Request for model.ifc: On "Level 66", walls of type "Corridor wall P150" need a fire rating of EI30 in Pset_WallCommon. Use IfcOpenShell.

First a look at what the model holds.

```python
import ifcopenshell
import ifcopenshell.util.element

model = ifcopenshell.open("model.ifc")
print(model.schema)
storey = next(s for s in model.by_type("IfcBuildingStorey") if s.Name == "Level 66")
walls = [e for e in ifcopenshell.util.element.get_decomposition(storey) if e.is_a("IfcWall")]
seen = {}
for e in walls:
    element_type = ifcopenshell.util.element.get_type(e)
    key = (element_type.Name if element_type != e and element_type else None, ifcopenshell.util.element.get_pset(e, "Pset_WallCommon", "FireRating"))
    seen[key] = seen.get(key, 0) + 1
for (name, value), count in sorted(seen.items(), key=str):
    print(count, "x", name, "|", value)
```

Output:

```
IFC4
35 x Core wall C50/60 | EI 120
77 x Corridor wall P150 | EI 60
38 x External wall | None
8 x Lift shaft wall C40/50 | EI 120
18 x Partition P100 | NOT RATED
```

```python
import ifcopenshell
import ifcopenshell.api.pset
import ifcopenshell.util.element

model = ifcopenshell.open("model.ifc")

storey = next(s for s in model.by_type("IfcBuildingStorey") if s.Name == "Level 66")
walls = [e for e in ifcopenshell.util.element.get_decomposition(storey) if e.is_a("IfcWall")]

count = 0
for e in walls:
    element_type = ifcopenshell.util.element.get_type(e)
    if element_type in (None, e) or element_type.Name != "Corridor wall P150":
        continue
    found = ifcopenshell.util.element.get_pset(e, "Pset_WallCommon", should_inherit=False)
    if found:
        pset = model.by_id(found["id"])
        if len(ifcopenshell.util.element.get_elements_by_pset(pset)) > 1:
            pset = ifcopenshell.api.pset.unshare_pset(model, products=[e], pset=pset)[0]
    else:
        pset = ifcopenshell.api.pset.add_pset(model, product=e, name="Pset_WallCommon")
    ifcopenshell.api.pset.edit_pset(model, pset=pset, properties={"FireRating": "EI30"})
    count += 1

print(count, "walls updated")

model.write("model_v2.ifc")
```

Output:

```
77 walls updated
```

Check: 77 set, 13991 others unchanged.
